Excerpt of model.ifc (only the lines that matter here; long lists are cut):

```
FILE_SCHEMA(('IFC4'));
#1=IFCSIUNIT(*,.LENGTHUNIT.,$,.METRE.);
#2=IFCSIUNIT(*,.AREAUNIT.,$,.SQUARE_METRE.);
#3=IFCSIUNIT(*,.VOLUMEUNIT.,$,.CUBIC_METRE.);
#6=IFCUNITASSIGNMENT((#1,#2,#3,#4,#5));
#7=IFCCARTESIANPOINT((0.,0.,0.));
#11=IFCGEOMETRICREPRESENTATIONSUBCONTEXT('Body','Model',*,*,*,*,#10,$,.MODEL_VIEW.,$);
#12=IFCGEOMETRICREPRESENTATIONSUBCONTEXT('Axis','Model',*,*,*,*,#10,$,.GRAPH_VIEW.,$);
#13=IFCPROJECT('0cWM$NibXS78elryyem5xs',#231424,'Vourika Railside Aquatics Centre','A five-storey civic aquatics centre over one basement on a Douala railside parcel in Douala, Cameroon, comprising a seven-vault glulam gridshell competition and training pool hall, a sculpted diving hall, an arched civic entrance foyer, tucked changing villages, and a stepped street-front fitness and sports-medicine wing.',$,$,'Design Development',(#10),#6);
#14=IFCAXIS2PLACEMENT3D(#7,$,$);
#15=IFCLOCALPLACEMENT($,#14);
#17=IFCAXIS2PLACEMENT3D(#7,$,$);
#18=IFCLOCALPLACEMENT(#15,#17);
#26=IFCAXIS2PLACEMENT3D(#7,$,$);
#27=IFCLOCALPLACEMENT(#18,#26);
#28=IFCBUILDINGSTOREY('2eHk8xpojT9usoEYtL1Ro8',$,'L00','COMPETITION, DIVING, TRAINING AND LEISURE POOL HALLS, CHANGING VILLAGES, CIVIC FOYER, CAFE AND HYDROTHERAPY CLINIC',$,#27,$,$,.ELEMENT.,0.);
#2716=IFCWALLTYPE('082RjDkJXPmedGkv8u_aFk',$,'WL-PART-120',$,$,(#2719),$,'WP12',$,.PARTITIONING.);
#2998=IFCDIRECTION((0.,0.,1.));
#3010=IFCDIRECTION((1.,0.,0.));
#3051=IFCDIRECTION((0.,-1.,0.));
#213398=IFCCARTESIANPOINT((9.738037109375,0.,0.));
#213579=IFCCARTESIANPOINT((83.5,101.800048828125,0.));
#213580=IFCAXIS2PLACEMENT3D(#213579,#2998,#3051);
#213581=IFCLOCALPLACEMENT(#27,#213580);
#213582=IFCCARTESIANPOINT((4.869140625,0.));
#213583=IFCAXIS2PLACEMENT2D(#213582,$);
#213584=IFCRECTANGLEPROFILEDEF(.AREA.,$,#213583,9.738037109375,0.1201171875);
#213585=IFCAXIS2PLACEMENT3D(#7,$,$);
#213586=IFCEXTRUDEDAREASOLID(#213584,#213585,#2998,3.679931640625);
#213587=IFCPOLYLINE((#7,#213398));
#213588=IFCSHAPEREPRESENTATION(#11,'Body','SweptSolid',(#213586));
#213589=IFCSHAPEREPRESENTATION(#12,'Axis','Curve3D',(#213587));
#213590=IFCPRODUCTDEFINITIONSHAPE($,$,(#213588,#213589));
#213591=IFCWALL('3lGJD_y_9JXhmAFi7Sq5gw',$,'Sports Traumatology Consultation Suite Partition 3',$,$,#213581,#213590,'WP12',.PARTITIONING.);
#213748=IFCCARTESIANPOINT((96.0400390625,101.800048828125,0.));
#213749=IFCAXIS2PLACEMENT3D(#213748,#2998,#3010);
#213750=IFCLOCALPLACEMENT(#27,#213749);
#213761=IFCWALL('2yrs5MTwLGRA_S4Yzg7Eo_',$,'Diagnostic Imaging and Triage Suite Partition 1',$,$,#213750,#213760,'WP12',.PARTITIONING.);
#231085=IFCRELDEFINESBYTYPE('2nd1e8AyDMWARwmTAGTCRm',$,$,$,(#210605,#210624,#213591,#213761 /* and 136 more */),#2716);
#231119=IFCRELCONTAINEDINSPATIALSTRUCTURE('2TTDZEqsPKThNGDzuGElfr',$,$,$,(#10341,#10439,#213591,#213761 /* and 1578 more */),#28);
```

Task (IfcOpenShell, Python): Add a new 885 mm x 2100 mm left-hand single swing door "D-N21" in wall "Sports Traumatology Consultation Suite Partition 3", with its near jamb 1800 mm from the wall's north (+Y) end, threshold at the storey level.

```python
import numpy as np
import ifcopenshell
import ifcopenshell.api.feature
import ifcopenshell.api.geometry
import ifcopenshell.api.root
import ifcopenshell.api.spatial
import ifcopenshell.geom
import ifcopenshell.util.element
import ifcopenshell.util.placement
import ifcopenshell.util.representation
import ifcopenshell.util.shape
import ifcopenshell.util.unit

model = ifcopenshell.open("model.ifc")
unit_scale = ifcopenshell.util.unit.calculate_unit_scale(model)
settings = ifcopenshell.geom.settings()


def volume(element):
    """Net volume in cubic metres, openings subtracted."""
    shape = ifcopenshell.geom.create_shape(settings, element)
    return ifcopenshell.util.shape.get_volume(shape.geometry)


wall = model.by_id(213591)
storey = ifcopenshell.util.element.get_container(wall, ifc_class="IfcBuildingStorey")
context = ifcopenshell.util.representation.get_context(model, "Model", "Body", "MODEL_VIEW")
before = volume(wall)

width, height, from_end, sill = 0.885, 2.1, 1.8, 0.0  # metres

# The wall runs along its own X axis, and the end named is its -X end.
wall_shape = ifcopenshell.geom.create_shape(settings, wall)
x, y, z = ifcopenshell.util.shape.get_vertices(wall_shape.geometry).T
start = x.min() + from_end
face, thickness = float(y.min()), float(y.max() - y.min())
wall_matrix = ifcopenshell.util.placement.get_local_placement(wall.ObjectPlacement)
level = ifcopenshell.util.placement.get_local_placement(storey.ObjectPlacement)[2, 3]


def in_wall(x, y):
    """Placement at x, y metres in the wall's axes, at sill height."""
    matrix = wall_matrix.copy()
    matrix[:, 3] = wall_matrix @ np.array([x / unit_scale, y / unit_scale, 0.0, 1.0])
    matrix[2, 3] = level + sill / unit_scale
    return matrix


# Opening: a box that overshoots both wall faces by 50 mm.
opening = ifcopenshell.api.root.create_entity(model, ifc_class="IfcOpeningElement", predefined_type="OPENING")
box = ifcopenshell.api.geometry.add_wall_representation(
    model, context=context, length=width, height=height, thickness=thickness + 0.1
)
ifcopenshell.api.geometry.assign_representation(model, product=opening, representation=box)
ifcopenshell.api.geometry.edit_object_placement(model, product=opening, matrix=in_wall(start, face - 0.05), is_si=False)
ifcopenshell.api.feature.add_feature(model, feature=opening, element=wall)

door = ifcopenshell.api.root.create_entity(model, ifc_class="IfcDoor", name="D-N21", predefined_type="DOOR")
door.OverallWidth, door.OverallHeight = width / unit_scale, height / unit_scale
door.OperationType = "SINGLE_SWING_LEFT"
body = ifcopenshell.api.geometry.add_door_representation(
    model,
    context=context,
    overall_width=door.OverallWidth,
    overall_height=door.OverallHeight,
    operation_type="SINGLE_SWING_LEFT",
    lining_properties={"LiningDepth": thickness / unit_scale, "ThresholdDepth": thickness / unit_scale},
)
ifcopenshell.api.geometry.assign_representation(model, product=door, representation=body)
ifcopenshell.api.spatial.assign_container(model, products=[door], relating_structure=storey)
ifcopenshell.api.feature.add_filling(model, opening=opening, element=door)

# The lining spans the wall, so the door starts at the wall face.
ifcopenshell.api.geometry.edit_object_placement(model, product=door, matrix=in_wall(start, face), is_si=False)

after = volume(wall)

print(f"wall volume {before:.3f} -> {after:.3f} m3")

model.write("model_edited.ifc")
```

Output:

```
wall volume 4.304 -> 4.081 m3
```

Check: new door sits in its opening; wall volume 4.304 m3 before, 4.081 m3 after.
